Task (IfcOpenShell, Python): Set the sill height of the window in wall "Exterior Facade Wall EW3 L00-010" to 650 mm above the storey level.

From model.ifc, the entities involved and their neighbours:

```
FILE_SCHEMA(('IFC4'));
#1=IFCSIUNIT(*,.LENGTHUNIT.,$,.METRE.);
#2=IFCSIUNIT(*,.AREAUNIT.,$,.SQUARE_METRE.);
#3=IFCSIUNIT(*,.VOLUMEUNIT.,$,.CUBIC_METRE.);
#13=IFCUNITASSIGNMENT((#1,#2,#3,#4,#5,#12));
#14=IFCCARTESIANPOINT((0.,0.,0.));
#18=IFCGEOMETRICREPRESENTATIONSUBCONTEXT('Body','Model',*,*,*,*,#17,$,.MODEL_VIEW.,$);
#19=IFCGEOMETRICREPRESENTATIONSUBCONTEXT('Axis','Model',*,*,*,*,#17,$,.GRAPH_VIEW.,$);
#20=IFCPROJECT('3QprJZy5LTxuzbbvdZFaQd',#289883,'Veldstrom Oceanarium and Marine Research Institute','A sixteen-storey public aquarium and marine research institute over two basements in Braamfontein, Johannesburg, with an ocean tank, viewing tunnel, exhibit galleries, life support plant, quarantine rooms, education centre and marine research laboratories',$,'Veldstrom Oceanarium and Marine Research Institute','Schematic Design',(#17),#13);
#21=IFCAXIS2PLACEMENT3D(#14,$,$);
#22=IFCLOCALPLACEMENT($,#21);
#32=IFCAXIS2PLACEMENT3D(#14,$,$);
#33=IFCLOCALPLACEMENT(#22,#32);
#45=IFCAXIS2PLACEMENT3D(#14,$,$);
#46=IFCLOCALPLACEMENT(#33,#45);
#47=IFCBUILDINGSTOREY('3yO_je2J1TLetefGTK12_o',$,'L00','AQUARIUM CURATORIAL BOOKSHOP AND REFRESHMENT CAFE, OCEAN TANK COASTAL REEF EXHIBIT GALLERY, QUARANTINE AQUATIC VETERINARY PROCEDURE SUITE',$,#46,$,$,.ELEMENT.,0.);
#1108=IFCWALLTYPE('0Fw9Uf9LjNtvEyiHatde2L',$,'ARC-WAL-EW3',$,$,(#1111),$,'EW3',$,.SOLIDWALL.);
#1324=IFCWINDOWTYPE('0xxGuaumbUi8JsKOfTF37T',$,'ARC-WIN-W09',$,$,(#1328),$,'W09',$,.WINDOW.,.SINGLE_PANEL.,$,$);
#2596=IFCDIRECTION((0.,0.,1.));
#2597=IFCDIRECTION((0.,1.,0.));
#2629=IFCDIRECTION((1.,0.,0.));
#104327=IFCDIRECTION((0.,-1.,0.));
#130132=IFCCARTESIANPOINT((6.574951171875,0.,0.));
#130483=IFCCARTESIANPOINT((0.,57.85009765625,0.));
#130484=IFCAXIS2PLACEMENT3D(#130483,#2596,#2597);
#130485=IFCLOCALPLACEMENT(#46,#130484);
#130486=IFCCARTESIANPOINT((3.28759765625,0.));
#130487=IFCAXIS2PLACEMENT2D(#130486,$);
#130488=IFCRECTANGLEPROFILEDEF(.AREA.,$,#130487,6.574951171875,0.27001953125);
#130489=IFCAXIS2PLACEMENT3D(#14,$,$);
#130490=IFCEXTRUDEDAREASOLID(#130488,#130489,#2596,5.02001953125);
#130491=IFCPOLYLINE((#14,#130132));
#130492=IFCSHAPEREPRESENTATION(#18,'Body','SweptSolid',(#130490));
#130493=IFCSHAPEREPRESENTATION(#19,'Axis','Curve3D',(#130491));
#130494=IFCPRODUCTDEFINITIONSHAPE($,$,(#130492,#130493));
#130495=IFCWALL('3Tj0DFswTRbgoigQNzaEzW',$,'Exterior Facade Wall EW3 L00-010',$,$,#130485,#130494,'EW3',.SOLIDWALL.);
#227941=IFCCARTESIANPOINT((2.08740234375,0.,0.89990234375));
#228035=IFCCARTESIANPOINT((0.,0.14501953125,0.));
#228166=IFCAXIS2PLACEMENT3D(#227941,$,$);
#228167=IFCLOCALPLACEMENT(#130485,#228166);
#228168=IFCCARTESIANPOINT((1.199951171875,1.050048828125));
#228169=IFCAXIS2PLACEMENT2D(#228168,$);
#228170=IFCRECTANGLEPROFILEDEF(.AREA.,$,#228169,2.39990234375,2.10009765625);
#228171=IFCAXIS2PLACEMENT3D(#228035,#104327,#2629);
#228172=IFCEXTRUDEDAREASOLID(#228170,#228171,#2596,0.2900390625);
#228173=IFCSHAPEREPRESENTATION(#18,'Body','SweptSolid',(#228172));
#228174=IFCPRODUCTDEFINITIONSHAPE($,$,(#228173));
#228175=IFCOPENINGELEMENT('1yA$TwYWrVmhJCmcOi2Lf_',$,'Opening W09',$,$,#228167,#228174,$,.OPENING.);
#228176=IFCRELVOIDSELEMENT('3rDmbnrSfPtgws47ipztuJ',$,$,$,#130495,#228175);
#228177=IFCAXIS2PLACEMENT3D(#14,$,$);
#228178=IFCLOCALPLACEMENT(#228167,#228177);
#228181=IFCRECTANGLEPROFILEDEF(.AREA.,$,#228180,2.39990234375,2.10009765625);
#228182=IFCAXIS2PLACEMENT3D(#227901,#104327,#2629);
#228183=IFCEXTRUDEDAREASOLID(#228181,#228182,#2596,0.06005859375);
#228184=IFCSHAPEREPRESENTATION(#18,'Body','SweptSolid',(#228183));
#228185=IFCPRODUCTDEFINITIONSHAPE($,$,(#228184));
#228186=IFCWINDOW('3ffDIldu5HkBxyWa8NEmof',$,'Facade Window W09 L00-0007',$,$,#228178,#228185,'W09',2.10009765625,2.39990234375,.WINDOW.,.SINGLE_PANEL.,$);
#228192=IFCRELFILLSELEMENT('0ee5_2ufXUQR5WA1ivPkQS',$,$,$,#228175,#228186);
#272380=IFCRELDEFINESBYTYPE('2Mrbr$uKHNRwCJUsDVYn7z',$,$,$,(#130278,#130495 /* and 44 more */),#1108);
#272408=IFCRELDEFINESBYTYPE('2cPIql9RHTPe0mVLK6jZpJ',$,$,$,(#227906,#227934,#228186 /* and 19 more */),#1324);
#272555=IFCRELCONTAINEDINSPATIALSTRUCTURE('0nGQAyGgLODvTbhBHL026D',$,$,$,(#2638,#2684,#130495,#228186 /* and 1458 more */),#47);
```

```python
import numpy as np
import ifcopenshell
import ifcopenshell.api.geometry
import ifcopenshell.geom
import ifcopenshell.util.element
import ifcopenshell.util.placement
import ifcopenshell.util.shape
import ifcopenshell.util.unit

model = ifcopenshell.open("model.ifc")
unit_scale = ifcopenshell.util.unit.calculate_unit_scale(model)

window = model.by_id(228186)
opening = window.FillsVoids[0].RelatingOpeningElement
storey = ifcopenshell.util.element.get_container(window, ifc_class="IfcBuildingStorey")
level = ifcopenshell.util.placement.get_local_placement(storey.ObjectPlacement)[2, 3]

# The opening's origin need not be at the sill, so measure its lowest point.
shape = ifcopenshell.geom.create_shape(ifcopenshell.geom.settings(), opening)
bottom = ifcopenshell.util.shape.get_shape_bottom_elevation(shape, shape.geometry) / unit_scale
dz = level + 0.65 / unit_scale - bottom

shift = np.array([0.0, 0.0, dz])
# The window is placed relative to its opening, so it follows when the opening moves.
matrix = ifcopenshell.util.placement.get_local_placement(opening.ObjectPlacement)
matrix[:3, 3] += shift
ifcopenshell.api.geometry.edit_object_placement(
    model, product=opening, matrix=matrix, is_si=False, should_transform_children=True
)

print(f"moved by {dz * unit_scale:+.3f} m")

model.write("model_rev.ifc")
```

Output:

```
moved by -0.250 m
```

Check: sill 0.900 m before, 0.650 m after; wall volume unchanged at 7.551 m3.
